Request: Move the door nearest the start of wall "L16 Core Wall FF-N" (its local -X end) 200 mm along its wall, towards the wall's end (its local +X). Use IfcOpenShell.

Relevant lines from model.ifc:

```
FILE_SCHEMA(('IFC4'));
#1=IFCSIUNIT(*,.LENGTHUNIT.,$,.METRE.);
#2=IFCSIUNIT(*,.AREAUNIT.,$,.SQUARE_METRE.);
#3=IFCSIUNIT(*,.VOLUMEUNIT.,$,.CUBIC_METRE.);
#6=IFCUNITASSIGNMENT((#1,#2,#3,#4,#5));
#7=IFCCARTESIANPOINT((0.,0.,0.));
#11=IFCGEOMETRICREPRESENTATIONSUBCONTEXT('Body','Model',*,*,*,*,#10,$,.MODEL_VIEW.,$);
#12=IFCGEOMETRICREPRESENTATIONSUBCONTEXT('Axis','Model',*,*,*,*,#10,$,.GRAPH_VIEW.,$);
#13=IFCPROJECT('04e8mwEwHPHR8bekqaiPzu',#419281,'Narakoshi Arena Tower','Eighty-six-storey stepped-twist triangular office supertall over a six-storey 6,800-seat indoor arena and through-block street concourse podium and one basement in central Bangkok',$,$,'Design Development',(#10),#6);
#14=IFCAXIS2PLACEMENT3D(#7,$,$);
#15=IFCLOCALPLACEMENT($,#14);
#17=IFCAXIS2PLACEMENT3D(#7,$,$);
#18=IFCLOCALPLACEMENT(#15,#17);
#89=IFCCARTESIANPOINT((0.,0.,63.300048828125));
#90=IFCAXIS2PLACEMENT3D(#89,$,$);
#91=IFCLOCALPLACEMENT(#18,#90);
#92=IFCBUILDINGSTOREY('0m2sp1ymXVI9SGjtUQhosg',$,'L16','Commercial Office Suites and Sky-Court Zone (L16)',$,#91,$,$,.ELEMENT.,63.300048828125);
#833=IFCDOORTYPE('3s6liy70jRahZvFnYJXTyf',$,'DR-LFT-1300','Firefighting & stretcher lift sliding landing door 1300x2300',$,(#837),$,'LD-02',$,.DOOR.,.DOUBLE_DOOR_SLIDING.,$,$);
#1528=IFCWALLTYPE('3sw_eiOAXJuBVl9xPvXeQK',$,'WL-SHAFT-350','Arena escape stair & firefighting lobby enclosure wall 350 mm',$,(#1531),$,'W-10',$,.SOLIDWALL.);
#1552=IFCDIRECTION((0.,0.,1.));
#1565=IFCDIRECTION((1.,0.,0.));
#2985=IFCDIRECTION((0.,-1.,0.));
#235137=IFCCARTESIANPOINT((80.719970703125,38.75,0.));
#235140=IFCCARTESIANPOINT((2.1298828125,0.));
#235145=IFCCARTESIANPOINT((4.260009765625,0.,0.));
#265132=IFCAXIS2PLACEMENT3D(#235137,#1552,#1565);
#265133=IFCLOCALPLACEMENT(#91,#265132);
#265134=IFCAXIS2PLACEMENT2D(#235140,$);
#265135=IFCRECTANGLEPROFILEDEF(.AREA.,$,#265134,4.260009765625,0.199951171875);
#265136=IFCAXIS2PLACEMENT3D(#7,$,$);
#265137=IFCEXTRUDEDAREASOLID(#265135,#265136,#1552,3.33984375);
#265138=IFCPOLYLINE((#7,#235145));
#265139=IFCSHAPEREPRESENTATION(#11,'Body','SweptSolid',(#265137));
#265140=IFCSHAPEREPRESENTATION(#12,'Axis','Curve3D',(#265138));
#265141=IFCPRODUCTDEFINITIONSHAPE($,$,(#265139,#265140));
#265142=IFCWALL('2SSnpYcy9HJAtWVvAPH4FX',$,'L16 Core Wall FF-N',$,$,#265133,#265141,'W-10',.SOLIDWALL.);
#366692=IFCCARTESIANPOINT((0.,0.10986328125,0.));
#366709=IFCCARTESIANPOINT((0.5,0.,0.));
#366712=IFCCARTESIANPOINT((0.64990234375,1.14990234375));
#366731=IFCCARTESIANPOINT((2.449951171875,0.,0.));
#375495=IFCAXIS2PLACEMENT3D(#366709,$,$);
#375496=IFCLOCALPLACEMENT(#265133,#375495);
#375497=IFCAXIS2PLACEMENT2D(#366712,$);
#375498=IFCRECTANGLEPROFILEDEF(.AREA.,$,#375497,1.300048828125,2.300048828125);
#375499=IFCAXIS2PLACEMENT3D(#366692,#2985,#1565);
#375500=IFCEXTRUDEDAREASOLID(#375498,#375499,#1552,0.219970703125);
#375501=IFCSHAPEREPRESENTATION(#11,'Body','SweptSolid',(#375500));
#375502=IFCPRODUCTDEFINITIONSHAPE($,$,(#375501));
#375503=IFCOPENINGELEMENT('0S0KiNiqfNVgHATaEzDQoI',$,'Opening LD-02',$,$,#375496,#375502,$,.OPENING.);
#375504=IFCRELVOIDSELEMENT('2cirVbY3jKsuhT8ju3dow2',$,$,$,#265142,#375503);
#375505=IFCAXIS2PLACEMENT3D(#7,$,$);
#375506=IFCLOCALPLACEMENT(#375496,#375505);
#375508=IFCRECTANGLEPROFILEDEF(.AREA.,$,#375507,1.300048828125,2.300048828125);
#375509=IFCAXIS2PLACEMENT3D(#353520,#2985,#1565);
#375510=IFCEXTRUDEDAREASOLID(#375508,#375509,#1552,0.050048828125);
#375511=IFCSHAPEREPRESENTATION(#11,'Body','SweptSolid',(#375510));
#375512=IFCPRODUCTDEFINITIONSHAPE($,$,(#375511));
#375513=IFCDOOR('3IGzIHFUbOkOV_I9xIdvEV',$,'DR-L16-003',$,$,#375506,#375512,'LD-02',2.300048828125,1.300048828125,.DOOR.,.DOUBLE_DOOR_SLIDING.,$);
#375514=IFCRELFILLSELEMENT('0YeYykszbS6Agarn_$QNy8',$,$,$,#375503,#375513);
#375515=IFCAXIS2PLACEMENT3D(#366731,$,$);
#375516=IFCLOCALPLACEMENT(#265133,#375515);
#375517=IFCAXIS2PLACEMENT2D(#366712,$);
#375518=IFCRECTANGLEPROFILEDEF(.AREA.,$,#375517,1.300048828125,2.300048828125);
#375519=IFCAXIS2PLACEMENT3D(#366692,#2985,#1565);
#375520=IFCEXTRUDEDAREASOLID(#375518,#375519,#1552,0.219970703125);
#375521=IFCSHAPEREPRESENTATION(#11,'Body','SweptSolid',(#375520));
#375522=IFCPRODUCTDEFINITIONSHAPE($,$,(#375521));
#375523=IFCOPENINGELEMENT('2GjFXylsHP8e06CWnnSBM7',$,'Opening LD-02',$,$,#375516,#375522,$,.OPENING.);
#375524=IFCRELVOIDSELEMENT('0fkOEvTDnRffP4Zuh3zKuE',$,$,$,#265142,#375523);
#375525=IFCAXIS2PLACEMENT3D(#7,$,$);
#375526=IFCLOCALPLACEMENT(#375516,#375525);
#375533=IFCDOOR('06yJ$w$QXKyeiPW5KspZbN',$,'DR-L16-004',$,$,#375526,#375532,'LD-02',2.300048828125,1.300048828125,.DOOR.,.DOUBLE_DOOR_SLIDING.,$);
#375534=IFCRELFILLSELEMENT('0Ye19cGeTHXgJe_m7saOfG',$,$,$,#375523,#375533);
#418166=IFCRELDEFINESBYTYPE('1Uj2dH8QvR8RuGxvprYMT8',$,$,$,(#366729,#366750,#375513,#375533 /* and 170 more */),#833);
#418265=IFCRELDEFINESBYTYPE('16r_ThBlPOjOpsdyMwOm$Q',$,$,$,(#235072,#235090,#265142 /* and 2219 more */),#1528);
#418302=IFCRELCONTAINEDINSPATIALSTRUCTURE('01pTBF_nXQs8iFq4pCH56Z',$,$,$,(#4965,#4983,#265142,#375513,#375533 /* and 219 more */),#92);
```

```python
import ifcopenshell
import ifcopenshell.api.geometry
import ifcopenshell.util.placement
import ifcopenshell.util.unit

model = ifcopenshell.open("model.ifc")
unit_scale = ifcopenshell.util.unit.calculate_unit_scale(model)

door = model.by_id(375513)
opening = door.FillsVoids[0].RelatingOpeningElement
wall = opening.VoidsElements[0].RelatingBuildingElement

wall_matrix = ifcopenshell.util.placement.get_local_placement(wall.ObjectPlacement)
shift = wall_matrix[:3, 0] * 0.2 / unit_scale
before = ifcopenshell.util.placement.get_local_placement(door.ObjectPlacement)[:3, 3].copy()

# The door is placed relative to its opening, so it follows when the opening moves.
matrix = ifcopenshell.util.placement.get_local_placement(opening.ObjectPlacement)
matrix[:3, 3] += shift
ifcopenshell.api.geometry.edit_object_placement(
    model, product=opening, matrix=matrix, is_si=False, should_transform_children=True
)

after = ifcopenshell.util.placement.get_local_placement(door.ObjectPlacement)[:3, 3]
print("door moved by", (after - before).round(3) + 0.0)

model.write("model-out.ifc")
```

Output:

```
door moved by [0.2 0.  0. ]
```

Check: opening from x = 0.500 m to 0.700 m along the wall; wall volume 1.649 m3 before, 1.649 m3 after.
